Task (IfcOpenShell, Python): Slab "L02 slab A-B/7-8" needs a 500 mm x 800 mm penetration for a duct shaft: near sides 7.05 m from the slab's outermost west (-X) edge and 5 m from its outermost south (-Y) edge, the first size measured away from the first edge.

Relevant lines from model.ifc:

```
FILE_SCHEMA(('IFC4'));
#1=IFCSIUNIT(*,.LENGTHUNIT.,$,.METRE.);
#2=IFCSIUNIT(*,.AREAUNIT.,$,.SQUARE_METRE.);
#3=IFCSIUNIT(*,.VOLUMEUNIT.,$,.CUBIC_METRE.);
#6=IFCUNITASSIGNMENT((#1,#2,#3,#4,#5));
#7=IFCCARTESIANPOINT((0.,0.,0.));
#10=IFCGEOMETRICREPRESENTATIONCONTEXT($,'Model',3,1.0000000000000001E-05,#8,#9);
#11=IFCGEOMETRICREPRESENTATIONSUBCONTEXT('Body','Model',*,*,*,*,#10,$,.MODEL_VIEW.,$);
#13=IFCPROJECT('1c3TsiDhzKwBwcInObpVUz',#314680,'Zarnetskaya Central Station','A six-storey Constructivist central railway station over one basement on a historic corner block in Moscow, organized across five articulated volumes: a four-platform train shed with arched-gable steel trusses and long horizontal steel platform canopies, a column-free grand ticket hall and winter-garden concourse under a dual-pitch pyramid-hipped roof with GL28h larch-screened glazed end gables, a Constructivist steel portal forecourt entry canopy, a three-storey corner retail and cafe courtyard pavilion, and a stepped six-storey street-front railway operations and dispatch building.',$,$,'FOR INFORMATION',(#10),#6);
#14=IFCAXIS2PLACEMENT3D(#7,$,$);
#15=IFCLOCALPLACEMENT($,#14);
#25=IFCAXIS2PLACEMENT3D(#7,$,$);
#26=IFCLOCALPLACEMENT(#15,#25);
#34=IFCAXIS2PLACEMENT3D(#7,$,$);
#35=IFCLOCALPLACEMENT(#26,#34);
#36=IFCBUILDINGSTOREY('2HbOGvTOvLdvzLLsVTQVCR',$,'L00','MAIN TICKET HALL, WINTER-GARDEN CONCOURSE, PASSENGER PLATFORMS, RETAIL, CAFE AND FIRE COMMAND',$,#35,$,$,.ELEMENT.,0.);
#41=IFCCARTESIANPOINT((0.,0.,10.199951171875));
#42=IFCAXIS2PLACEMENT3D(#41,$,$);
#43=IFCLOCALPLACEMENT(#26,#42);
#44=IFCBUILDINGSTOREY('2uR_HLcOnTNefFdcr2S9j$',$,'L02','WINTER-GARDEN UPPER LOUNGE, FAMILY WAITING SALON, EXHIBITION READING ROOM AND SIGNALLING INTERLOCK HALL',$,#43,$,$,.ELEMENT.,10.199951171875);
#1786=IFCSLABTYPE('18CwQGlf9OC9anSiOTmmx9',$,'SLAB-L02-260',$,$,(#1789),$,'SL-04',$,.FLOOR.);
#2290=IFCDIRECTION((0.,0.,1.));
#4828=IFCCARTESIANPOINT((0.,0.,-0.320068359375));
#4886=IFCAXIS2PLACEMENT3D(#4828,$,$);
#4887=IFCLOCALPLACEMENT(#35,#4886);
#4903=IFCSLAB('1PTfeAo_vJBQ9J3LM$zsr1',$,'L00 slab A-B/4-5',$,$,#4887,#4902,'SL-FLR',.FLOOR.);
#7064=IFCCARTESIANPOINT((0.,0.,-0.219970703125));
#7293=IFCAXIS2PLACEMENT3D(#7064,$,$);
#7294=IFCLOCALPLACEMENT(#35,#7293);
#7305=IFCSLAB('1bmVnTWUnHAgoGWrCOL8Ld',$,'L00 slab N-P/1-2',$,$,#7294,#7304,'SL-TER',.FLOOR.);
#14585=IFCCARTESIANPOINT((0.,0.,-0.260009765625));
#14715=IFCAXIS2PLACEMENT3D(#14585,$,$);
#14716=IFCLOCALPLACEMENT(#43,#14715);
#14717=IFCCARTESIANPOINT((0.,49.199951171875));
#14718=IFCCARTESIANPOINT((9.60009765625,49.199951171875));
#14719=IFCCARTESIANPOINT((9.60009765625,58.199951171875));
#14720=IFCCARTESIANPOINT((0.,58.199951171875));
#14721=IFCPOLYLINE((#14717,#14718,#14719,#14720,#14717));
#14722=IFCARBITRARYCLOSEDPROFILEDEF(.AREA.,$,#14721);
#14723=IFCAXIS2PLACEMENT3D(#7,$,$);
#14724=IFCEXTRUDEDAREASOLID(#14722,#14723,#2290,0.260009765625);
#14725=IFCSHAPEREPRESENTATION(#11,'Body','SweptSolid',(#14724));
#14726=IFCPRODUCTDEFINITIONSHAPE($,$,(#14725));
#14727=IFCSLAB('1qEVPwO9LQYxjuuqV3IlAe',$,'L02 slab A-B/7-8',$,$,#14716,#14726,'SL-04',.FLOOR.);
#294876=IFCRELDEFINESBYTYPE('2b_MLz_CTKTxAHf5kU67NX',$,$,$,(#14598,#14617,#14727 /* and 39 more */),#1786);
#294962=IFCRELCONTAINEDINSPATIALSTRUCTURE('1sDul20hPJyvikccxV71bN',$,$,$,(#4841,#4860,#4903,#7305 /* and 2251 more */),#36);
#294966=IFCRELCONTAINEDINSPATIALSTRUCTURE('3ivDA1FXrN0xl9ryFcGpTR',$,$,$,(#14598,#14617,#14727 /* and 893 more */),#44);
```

```python
import numpy as np
import ifcopenshell
import ifcopenshell.api.feature
import ifcopenshell.api.geometry
import ifcopenshell.api.root
import ifcopenshell.geom
import ifcopenshell.util.placement
import ifcopenshell.util.representation
import ifcopenshell.util.shape
import ifcopenshell.util.unit

model = ifcopenshell.open("model.ifc")
unit_scale = ifcopenshell.util.unit.calculate_unit_scale(model)
settings = ifcopenshell.geom.settings()


def volume(element):
    """Net volume in cubic metres, openings subtracted."""
    shape = ifcopenshell.geom.create_shape(settings, element)
    return ifcopenshell.util.shape.get_volume(shape.geometry)


slab = model.by_id(14727)
before = volume(slab)

# Extent in the slab's own axes, in metres. The edges named are its -X and -Y sides.
slab_shape = ifcopenshell.geom.create_shape(settings, slab)
vertices = ifcopenshell.util.shape.get_vertices(slab_shape.geometry)
x_min, y_min, bottom = vertices.min(axis=0)
top = vertices[:, 2].max()

opening = ifcopenshell.api.root.create_entity(model, ifc_class="IfcOpeningElement", name="Duct shaft opening", predefined_type="OPENING")
context = ifcopenshell.util.representation.get_context(model, "Model", "Body", "MODEL_VIEW")
width, depth = 0.5, 0.8
outline = [(0.0, 0.0), (width, 0.0), (width, depth), (0.0, depth), (0.0, 0.0)]
# Overshoot both faces by 50 mm so the cut is clean.
shape = ifcopenshell.api.geometry.add_slab_representation(
    model, context=context, depth=top - bottom + 0.1, polyline=outline
)
ifcopenshell.api.geometry.assign_representation(model, product=opening, representation=shape)

matrix = ifcopenshell.util.placement.get_local_placement(slab.ObjectPlacement)
matrix[:, 3] = matrix @ np.append(np.array([x_min + 7.05, y_min + 5, bottom - 0.05]) / unit_scale, 1.0)
ifcopenshell.api.geometry.edit_object_placement(model, product=opening, matrix=matrix, is_si=False)
ifcopenshell.api.feature.add_feature(model, feature=opening, element=slab)

after = volume(slab)

print(f"slab volume {before:.3f} -> {after:.3f} m3")

model.write("model_edited.ifc")
```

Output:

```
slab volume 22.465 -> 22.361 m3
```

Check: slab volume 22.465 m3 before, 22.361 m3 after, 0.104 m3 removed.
